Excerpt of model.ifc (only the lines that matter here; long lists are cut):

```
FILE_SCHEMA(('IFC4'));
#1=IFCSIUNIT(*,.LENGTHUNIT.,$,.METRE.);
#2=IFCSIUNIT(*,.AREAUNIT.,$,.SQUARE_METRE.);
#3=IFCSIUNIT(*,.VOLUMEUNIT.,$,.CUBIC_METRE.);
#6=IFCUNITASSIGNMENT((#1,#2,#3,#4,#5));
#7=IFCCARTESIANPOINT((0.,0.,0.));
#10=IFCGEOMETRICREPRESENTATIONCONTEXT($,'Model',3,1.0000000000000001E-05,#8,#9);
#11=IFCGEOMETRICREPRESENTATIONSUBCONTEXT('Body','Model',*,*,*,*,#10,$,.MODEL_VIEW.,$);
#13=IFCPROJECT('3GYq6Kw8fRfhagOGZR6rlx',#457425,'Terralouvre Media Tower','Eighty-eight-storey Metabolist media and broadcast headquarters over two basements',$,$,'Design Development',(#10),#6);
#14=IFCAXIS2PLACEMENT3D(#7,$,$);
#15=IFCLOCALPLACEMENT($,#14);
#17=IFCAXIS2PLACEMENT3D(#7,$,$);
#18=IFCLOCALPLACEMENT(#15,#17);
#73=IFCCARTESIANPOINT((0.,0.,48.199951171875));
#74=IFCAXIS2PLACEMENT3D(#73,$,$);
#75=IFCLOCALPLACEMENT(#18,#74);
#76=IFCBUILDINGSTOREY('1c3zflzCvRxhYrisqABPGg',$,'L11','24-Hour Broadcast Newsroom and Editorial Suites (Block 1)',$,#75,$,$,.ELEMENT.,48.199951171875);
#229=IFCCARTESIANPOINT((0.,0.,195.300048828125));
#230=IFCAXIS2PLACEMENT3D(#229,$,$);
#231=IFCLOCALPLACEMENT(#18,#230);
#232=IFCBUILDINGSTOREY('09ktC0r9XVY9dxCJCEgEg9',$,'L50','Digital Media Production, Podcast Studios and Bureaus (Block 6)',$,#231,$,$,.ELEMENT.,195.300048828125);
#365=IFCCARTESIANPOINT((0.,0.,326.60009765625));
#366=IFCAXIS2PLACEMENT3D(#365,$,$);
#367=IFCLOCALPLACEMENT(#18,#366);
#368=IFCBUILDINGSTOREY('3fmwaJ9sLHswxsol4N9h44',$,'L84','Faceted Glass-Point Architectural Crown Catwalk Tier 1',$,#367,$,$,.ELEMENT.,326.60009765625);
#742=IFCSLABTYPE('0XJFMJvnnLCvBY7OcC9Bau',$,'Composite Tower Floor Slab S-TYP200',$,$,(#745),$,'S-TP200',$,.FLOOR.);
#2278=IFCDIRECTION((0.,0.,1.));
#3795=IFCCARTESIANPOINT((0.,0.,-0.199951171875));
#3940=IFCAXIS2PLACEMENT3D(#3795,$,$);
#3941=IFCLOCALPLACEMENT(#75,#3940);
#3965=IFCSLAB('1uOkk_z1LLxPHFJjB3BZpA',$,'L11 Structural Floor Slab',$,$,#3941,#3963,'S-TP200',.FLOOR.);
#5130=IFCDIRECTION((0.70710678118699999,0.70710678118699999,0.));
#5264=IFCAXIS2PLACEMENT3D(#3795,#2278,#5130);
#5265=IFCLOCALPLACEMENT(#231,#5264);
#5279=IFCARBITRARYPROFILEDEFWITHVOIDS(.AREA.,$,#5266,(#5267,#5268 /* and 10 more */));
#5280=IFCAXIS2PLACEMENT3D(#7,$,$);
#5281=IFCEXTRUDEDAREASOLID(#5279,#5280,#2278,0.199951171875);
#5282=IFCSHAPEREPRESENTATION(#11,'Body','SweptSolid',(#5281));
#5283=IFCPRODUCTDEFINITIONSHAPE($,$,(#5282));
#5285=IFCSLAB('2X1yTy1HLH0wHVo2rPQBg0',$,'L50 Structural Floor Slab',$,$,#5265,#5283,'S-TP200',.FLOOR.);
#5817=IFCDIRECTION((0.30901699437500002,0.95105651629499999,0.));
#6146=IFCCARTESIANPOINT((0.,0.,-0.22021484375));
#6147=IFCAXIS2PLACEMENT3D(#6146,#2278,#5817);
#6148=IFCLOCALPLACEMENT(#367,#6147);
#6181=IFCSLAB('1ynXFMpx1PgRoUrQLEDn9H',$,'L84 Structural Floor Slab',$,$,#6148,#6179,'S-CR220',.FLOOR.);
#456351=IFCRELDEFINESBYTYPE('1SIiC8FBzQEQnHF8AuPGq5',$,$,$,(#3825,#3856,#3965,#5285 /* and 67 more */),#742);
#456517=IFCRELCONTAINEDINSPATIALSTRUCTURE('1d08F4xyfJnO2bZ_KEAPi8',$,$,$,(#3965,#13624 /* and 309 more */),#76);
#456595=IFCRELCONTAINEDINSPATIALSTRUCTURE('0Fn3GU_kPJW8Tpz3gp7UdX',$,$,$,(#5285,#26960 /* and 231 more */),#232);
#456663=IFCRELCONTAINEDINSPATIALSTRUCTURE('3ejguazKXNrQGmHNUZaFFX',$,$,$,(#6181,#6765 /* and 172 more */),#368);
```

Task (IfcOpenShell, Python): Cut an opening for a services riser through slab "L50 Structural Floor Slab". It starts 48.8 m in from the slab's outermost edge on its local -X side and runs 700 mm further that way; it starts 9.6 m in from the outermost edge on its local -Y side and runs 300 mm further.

```python
import numpy as np
import ifcopenshell
import ifcopenshell.api.feature
import ifcopenshell.api.geometry
import ifcopenshell.api.root
import ifcopenshell.geom
import ifcopenshell.util.placement
import ifcopenshell.util.representation
import ifcopenshell.util.shape
import ifcopenshell.util.unit

model = ifcopenshell.open("model.ifc")
unit_scale = ifcopenshell.util.unit.calculate_unit_scale(model)
settings = ifcopenshell.geom.settings()


def volume(element):
    """Net volume in cubic metres, openings subtracted."""
    shape = ifcopenshell.geom.create_shape(settings, element)
    return ifcopenshell.util.shape.get_volume(shape.geometry)


slab = model.by_id(5285)
before = volume(slab)

# Extent in the slab's own axes, in metres. The edges named are its -X and -Y sides.
slab_shape = ifcopenshell.geom.create_shape(settings, slab)
vertices = ifcopenshell.util.shape.get_vertices(slab_shape.geometry)
x_min, y_min, bottom = vertices.min(axis=0)
top = vertices[:, 2].max()

opening = ifcopenshell.api.root.create_entity(model, ifc_class="IfcOpeningElement", name="Services riser opening", predefined_type="OPENING")
context = ifcopenshell.util.representation.get_context(model, "Model", "Body", "MODEL_VIEW")
width, depth = 0.7, 0.3
outline = [(0.0, 0.0), (width, 0.0), (width, depth), (0.0, depth), (0.0, 0.0)]
# Overshoot both faces by 50 mm so the cut is clean.
shape = ifcopenshell.api.geometry.add_slab_representation(
    model, context=context, depth=top - bottom + 0.1, polyline=outline
)
ifcopenshell.api.geometry.assign_representation(model, product=opening, representation=shape)

matrix = ifcopenshell.util.placement.get_local_placement(slab.ObjectPlacement)
matrix[:, 3] = matrix @ np.append(np.array([x_min + 48.8, y_min + 9.6, bottom - 0.05]) / unit_scale, 1.0)
ifcopenshell.api.geometry.edit_object_placement(model, product=opening, matrix=matrix, is_si=False)
ifcopenshell.api.feature.add_feature(model, feature=opening, element=slab)

after = volume(slab)

print(f"slab volume {before:.3f} -> {after:.3f} m3")

model.write("model-out.ifc")
```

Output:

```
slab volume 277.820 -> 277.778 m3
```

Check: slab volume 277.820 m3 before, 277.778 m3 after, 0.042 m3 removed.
